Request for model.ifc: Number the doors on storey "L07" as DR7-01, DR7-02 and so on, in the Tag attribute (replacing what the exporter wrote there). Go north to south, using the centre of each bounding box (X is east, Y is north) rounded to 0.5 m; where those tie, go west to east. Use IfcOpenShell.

First a look at what the model holds.

```python
import ifcopenshell
import ifcopenshell.util.element
import ifcopenshell.util.placement

model = ifcopenshell.open("model.ifc")
print(model.schema)
storey = next(s for s in model.by_type("IfcBuildingStorey") if s.Name == "L07")
doors = [e for e in ifcopenshell.util.element.get_decomposition(storey) if e.is_a("IfcDoor")]
for e in sorted(doors, key=lambda e: e.id()):
    origin = ifcopenshell.util.placement.get_local_placement(e.ObjectPlacement)[:3, 3]
    print(e.id(), e.Tag, e.Name, origin.round(2) + 0.0, sep=" | ")
```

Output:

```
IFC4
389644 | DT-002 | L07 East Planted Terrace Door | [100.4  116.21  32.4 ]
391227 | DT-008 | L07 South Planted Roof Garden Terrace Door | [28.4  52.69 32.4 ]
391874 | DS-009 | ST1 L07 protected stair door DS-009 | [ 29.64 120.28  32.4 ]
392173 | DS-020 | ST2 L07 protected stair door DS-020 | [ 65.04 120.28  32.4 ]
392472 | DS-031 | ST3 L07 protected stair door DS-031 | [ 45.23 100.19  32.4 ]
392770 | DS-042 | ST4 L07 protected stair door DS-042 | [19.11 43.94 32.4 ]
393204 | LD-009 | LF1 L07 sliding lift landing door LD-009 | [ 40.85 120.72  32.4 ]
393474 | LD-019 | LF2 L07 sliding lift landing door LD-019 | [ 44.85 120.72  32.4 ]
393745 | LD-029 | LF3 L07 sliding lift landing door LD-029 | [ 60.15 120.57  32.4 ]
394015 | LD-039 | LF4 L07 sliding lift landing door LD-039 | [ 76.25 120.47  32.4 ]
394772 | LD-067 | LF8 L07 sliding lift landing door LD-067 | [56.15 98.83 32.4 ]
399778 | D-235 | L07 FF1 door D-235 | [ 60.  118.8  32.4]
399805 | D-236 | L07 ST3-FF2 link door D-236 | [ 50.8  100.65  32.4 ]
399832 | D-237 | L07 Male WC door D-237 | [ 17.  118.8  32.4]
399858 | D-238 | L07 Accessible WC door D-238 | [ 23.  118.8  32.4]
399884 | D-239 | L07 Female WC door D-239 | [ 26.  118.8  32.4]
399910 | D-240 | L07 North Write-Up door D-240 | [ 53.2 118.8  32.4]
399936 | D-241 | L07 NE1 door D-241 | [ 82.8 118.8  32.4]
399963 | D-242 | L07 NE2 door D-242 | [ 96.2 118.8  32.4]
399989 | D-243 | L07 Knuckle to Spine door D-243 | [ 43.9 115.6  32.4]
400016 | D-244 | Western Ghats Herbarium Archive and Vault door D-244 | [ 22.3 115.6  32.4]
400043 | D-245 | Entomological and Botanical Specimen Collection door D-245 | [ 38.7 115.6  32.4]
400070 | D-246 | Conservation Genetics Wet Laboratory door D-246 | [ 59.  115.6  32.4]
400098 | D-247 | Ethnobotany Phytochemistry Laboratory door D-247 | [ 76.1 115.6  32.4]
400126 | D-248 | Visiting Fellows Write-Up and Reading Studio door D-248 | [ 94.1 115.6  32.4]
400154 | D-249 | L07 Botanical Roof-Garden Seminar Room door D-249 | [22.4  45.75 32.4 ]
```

```python
import ifcopenshell
import ifcopenshell.geom
import ifcopenshell.util.element
import ifcopenshell.util.shape

model = ifcopenshell.open("model.ifc")
settings = ifcopenshell.geom.settings()
settings.set("use-world-coords", True)


def centre(element):
    shape = ifcopenshell.geom.create_shape(settings, element)
    return ifcopenshell.util.shape.get_bbox_centroid(shape.geometry)


storey = next(s for s in model.by_type("IfcBuildingStorey") if s.Name == "L07")
doors = [e for e in ifcopenshell.util.element.get_decomposition(storey) if e.is_a("IfcDoor")]

# Insertion points can sit at a corner or the storey origin, so sort by the geometry (in metres).
centres = {e: centre(e) for e in doors}
doors.sort(key=lambda e: (-round(centres[e][1] / 0.5), centres[e][0]))

for i, e in enumerate(doors, start=1):
    number = f"DR7-{i:02d}"
    e.Tag = number
    print(e.id(), number)

model.write("model-out.ifc")
```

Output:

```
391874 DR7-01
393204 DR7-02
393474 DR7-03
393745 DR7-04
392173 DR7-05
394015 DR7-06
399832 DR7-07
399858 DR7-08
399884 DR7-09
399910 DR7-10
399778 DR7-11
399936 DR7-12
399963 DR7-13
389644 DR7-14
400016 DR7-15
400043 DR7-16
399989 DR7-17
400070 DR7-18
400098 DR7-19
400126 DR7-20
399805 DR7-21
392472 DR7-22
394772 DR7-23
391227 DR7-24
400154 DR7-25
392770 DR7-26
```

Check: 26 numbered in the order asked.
